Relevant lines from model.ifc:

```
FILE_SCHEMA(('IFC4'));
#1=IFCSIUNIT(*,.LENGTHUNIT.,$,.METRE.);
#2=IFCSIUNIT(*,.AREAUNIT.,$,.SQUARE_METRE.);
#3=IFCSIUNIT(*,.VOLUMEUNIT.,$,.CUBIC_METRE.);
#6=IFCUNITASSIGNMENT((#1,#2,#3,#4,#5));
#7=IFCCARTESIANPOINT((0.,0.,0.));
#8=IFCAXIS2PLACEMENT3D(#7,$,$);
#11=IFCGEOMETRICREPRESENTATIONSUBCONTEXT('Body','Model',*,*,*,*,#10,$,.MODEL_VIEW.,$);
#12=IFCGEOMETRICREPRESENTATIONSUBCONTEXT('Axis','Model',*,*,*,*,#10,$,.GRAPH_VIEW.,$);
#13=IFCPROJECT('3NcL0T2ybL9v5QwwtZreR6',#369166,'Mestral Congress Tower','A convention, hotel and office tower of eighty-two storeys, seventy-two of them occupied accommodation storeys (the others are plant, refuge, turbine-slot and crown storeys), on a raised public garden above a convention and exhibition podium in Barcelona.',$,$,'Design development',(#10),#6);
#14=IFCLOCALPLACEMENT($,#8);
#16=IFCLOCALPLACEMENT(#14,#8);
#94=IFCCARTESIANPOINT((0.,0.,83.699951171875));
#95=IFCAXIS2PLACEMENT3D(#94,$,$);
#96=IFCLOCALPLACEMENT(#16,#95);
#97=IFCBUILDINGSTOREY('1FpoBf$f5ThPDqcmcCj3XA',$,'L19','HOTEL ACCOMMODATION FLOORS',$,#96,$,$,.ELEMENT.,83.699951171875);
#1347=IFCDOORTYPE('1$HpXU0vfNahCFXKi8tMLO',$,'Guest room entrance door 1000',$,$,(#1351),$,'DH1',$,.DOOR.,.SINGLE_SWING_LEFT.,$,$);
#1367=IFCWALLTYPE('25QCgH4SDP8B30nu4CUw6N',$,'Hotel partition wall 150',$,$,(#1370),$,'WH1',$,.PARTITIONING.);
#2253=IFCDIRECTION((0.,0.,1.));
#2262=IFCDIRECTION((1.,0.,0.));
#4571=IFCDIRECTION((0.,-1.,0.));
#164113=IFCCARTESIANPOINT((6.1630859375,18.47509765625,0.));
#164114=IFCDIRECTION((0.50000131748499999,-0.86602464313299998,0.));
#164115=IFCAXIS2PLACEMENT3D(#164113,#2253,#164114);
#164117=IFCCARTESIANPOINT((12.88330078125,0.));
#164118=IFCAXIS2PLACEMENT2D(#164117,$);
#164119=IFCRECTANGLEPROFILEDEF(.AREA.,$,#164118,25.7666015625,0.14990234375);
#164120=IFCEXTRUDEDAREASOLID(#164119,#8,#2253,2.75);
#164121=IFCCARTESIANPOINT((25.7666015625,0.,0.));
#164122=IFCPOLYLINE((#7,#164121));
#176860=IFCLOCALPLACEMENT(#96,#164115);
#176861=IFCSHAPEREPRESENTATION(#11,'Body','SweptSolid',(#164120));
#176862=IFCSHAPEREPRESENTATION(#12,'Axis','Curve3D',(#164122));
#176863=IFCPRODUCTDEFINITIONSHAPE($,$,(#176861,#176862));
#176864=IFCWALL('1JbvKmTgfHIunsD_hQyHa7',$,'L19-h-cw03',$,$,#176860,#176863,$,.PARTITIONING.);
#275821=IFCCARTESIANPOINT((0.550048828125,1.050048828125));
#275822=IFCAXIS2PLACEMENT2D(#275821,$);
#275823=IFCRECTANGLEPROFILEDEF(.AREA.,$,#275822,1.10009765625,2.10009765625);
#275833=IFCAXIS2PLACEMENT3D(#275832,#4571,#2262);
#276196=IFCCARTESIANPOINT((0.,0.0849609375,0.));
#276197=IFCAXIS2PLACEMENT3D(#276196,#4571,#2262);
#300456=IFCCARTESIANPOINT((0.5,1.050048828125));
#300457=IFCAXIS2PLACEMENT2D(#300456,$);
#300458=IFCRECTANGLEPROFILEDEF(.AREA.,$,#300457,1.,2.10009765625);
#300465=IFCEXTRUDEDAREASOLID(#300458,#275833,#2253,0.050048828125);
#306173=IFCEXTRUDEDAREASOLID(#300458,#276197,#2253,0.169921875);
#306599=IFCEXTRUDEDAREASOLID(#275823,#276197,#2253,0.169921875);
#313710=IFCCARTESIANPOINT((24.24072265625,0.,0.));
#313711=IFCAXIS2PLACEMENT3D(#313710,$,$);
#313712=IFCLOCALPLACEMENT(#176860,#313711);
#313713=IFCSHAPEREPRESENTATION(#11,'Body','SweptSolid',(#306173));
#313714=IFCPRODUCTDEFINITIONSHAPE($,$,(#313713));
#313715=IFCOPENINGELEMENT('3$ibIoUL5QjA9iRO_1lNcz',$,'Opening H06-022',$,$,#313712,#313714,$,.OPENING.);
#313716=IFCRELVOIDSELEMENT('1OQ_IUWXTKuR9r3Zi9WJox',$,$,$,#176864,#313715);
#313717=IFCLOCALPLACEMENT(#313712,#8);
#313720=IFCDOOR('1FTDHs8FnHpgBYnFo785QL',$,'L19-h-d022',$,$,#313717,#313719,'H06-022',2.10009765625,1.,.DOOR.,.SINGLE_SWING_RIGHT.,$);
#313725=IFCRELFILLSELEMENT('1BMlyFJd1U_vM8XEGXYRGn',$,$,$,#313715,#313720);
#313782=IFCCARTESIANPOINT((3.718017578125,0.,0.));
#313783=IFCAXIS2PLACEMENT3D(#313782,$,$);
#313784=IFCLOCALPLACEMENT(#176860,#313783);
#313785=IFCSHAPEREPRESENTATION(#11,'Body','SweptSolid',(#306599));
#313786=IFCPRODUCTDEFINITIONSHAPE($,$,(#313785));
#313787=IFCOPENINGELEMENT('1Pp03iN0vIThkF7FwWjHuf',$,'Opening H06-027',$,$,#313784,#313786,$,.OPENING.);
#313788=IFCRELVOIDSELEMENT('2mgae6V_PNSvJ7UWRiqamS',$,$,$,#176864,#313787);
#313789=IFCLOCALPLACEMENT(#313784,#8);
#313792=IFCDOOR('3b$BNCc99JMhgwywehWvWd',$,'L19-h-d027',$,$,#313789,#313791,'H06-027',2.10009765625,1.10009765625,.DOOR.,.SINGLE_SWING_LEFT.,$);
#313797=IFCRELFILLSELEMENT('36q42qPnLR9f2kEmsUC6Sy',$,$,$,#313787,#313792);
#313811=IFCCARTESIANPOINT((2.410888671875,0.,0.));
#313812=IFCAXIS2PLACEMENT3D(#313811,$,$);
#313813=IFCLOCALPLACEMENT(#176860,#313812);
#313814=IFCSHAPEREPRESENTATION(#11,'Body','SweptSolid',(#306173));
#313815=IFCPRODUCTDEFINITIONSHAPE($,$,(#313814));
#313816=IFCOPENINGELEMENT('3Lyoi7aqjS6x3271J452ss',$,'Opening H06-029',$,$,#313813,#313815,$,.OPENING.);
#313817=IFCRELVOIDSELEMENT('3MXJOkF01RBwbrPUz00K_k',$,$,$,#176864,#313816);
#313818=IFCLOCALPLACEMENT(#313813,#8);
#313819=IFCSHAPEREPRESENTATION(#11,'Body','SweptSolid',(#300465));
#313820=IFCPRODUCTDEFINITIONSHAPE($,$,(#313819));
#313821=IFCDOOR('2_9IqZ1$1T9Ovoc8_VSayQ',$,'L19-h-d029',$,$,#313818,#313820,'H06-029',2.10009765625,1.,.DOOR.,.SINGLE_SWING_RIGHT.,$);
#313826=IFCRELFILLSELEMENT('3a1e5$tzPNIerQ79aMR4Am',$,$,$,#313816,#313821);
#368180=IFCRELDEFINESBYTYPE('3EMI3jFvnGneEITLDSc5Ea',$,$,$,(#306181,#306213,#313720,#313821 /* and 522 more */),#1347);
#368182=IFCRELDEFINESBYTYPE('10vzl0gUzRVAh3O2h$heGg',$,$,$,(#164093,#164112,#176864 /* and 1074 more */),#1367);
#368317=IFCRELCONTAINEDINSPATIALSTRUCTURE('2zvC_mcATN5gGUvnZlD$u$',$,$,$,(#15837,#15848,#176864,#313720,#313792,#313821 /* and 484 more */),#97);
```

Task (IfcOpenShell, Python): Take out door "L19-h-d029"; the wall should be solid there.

```python
import ifcopenshell
import ifcopenshell.api.feature
import ifcopenshell.api.root
import ifcopenshell.geom
import ifcopenshell.util.shape

model = ifcopenshell.open("model.ifc")
settings = ifcopenshell.geom.settings()


def volume(element):
    """Net volume in cubic metres, openings subtracted."""
    shape = ifcopenshell.geom.create_shape(settings, element)
    return ifcopenshell.util.shape.get_volume(shape.geometry)


door = model.by_guid("2_9IqZ1$1T9Ovoc8_VSayQ")
opening = door.FillsVoids[0].RelatingOpeningElement
wall = opening.VoidsElements[0].RelatingBuildingElement
before = volume(wall)

ifcopenshell.api.root.remove_product(model, product=door)
ifcopenshell.api.feature.remove_feature(model, feature=opening)

after = volume(wall)

print(f"wall volume {before:.3f} -> {after:.3f} m3")

model.write("model_rev.ifc")
```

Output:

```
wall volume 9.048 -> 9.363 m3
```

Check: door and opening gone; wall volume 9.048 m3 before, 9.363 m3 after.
